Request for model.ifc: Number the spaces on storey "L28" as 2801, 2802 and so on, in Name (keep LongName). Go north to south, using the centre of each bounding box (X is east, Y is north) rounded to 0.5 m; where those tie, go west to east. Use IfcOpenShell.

First a look at what the model holds.

```python
import ifcopenshell
import ifcopenshell.util.element
import ifcopenshell.util.placement

model = ifcopenshell.open("model.ifc")
print(model.schema)
storey = next(s for s in model.by_type("IfcBuildingStorey") if s.Name == "L28")
spaces = [e for e in ifcopenshell.util.element.get_decomposition(storey) if e.is_a("IfcSpace")]
for e in sorted(spaces, key=lambda e: e.id()):
    origin = ifcopenshell.util.placement.get_local_placement(e.ObjectPlacement)[:3, 3]
    print(e.id(), e.Name, e.LongName, origin.round(2) + 0.0, sep=" | ")
```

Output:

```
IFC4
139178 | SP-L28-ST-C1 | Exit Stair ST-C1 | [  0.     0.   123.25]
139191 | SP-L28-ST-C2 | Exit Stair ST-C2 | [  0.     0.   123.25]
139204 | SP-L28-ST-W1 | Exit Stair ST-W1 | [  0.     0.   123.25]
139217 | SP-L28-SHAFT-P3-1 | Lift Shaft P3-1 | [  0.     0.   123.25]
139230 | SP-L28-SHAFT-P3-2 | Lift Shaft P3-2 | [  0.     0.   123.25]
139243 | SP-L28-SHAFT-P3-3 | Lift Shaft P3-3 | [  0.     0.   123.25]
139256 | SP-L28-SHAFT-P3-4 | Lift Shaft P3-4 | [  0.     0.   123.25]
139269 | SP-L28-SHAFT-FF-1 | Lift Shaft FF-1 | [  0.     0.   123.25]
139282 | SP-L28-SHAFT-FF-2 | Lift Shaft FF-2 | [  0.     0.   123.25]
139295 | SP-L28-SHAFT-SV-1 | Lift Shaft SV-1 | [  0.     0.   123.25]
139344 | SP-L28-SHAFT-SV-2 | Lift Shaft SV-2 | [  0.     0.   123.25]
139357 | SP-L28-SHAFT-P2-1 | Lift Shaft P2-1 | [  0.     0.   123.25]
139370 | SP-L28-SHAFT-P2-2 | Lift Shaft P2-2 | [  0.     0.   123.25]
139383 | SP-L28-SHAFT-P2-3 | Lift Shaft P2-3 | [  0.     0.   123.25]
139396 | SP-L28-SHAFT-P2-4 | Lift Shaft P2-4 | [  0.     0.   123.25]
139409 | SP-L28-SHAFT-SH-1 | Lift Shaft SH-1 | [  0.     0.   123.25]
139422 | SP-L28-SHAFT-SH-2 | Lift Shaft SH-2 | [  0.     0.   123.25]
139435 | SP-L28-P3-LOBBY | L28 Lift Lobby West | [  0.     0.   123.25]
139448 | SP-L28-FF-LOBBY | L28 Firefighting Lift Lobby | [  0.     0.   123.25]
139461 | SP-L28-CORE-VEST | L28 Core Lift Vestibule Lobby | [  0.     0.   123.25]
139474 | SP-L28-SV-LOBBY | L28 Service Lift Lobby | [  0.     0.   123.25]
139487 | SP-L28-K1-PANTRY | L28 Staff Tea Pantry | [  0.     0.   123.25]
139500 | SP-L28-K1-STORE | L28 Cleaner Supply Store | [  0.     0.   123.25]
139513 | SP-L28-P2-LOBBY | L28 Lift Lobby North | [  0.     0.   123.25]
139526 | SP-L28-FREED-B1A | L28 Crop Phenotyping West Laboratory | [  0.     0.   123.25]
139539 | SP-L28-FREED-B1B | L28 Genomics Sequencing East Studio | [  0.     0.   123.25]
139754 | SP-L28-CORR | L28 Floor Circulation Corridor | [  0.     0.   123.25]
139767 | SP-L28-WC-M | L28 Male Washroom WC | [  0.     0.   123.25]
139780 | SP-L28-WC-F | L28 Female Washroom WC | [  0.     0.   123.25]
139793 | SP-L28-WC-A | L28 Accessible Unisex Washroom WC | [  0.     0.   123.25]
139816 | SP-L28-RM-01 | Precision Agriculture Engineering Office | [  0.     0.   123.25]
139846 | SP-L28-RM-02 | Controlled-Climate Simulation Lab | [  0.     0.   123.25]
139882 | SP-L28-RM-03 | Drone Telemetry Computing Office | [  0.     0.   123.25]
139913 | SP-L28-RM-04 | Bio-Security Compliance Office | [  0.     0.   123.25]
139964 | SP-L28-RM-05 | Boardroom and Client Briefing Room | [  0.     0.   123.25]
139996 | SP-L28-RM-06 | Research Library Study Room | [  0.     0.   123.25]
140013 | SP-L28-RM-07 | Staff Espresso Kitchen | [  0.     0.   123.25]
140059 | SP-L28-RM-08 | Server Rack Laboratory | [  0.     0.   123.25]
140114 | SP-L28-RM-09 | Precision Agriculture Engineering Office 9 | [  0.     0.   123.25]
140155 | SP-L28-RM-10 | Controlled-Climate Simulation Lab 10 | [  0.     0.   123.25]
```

```python
import ifcopenshell
import ifcopenshell.geom
import ifcopenshell.util.element
import ifcopenshell.util.shape

model = ifcopenshell.open("model.ifc")
settings = ifcopenshell.geom.settings()
settings.set("use-world-coords", True)


def centre(element):
    shape = ifcopenshell.geom.create_shape(settings, element)
    return ifcopenshell.util.shape.get_bbox_centroid(shape.geometry)


storey = next(s for s in model.by_type("IfcBuildingStorey") if s.Name == "L28")
spaces = [e for e in ifcopenshell.util.element.get_decomposition(storey) if e.is_a("IfcSpace")]

# Insertion points can sit at a corner or the storey origin, so sort by the geometry (in metres).
centres = {e: centre(e) for e in spaces}
spaces.sort(key=lambda e: (-round(centres[e][1] / 0.5), centres[e][0]))

for i, e in enumerate(spaces, start=1):
    number = f"28{i:02d}"
    e.Name = number
    print(e.id(), number)

model.write("model_edited.ifc")
```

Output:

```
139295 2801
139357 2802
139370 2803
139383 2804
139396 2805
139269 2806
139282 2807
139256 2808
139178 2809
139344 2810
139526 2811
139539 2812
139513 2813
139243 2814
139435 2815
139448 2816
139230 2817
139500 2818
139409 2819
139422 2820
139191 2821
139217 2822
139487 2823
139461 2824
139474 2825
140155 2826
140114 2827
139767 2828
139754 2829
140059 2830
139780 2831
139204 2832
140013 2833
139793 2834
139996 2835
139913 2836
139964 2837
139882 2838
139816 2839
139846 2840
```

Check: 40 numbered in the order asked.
